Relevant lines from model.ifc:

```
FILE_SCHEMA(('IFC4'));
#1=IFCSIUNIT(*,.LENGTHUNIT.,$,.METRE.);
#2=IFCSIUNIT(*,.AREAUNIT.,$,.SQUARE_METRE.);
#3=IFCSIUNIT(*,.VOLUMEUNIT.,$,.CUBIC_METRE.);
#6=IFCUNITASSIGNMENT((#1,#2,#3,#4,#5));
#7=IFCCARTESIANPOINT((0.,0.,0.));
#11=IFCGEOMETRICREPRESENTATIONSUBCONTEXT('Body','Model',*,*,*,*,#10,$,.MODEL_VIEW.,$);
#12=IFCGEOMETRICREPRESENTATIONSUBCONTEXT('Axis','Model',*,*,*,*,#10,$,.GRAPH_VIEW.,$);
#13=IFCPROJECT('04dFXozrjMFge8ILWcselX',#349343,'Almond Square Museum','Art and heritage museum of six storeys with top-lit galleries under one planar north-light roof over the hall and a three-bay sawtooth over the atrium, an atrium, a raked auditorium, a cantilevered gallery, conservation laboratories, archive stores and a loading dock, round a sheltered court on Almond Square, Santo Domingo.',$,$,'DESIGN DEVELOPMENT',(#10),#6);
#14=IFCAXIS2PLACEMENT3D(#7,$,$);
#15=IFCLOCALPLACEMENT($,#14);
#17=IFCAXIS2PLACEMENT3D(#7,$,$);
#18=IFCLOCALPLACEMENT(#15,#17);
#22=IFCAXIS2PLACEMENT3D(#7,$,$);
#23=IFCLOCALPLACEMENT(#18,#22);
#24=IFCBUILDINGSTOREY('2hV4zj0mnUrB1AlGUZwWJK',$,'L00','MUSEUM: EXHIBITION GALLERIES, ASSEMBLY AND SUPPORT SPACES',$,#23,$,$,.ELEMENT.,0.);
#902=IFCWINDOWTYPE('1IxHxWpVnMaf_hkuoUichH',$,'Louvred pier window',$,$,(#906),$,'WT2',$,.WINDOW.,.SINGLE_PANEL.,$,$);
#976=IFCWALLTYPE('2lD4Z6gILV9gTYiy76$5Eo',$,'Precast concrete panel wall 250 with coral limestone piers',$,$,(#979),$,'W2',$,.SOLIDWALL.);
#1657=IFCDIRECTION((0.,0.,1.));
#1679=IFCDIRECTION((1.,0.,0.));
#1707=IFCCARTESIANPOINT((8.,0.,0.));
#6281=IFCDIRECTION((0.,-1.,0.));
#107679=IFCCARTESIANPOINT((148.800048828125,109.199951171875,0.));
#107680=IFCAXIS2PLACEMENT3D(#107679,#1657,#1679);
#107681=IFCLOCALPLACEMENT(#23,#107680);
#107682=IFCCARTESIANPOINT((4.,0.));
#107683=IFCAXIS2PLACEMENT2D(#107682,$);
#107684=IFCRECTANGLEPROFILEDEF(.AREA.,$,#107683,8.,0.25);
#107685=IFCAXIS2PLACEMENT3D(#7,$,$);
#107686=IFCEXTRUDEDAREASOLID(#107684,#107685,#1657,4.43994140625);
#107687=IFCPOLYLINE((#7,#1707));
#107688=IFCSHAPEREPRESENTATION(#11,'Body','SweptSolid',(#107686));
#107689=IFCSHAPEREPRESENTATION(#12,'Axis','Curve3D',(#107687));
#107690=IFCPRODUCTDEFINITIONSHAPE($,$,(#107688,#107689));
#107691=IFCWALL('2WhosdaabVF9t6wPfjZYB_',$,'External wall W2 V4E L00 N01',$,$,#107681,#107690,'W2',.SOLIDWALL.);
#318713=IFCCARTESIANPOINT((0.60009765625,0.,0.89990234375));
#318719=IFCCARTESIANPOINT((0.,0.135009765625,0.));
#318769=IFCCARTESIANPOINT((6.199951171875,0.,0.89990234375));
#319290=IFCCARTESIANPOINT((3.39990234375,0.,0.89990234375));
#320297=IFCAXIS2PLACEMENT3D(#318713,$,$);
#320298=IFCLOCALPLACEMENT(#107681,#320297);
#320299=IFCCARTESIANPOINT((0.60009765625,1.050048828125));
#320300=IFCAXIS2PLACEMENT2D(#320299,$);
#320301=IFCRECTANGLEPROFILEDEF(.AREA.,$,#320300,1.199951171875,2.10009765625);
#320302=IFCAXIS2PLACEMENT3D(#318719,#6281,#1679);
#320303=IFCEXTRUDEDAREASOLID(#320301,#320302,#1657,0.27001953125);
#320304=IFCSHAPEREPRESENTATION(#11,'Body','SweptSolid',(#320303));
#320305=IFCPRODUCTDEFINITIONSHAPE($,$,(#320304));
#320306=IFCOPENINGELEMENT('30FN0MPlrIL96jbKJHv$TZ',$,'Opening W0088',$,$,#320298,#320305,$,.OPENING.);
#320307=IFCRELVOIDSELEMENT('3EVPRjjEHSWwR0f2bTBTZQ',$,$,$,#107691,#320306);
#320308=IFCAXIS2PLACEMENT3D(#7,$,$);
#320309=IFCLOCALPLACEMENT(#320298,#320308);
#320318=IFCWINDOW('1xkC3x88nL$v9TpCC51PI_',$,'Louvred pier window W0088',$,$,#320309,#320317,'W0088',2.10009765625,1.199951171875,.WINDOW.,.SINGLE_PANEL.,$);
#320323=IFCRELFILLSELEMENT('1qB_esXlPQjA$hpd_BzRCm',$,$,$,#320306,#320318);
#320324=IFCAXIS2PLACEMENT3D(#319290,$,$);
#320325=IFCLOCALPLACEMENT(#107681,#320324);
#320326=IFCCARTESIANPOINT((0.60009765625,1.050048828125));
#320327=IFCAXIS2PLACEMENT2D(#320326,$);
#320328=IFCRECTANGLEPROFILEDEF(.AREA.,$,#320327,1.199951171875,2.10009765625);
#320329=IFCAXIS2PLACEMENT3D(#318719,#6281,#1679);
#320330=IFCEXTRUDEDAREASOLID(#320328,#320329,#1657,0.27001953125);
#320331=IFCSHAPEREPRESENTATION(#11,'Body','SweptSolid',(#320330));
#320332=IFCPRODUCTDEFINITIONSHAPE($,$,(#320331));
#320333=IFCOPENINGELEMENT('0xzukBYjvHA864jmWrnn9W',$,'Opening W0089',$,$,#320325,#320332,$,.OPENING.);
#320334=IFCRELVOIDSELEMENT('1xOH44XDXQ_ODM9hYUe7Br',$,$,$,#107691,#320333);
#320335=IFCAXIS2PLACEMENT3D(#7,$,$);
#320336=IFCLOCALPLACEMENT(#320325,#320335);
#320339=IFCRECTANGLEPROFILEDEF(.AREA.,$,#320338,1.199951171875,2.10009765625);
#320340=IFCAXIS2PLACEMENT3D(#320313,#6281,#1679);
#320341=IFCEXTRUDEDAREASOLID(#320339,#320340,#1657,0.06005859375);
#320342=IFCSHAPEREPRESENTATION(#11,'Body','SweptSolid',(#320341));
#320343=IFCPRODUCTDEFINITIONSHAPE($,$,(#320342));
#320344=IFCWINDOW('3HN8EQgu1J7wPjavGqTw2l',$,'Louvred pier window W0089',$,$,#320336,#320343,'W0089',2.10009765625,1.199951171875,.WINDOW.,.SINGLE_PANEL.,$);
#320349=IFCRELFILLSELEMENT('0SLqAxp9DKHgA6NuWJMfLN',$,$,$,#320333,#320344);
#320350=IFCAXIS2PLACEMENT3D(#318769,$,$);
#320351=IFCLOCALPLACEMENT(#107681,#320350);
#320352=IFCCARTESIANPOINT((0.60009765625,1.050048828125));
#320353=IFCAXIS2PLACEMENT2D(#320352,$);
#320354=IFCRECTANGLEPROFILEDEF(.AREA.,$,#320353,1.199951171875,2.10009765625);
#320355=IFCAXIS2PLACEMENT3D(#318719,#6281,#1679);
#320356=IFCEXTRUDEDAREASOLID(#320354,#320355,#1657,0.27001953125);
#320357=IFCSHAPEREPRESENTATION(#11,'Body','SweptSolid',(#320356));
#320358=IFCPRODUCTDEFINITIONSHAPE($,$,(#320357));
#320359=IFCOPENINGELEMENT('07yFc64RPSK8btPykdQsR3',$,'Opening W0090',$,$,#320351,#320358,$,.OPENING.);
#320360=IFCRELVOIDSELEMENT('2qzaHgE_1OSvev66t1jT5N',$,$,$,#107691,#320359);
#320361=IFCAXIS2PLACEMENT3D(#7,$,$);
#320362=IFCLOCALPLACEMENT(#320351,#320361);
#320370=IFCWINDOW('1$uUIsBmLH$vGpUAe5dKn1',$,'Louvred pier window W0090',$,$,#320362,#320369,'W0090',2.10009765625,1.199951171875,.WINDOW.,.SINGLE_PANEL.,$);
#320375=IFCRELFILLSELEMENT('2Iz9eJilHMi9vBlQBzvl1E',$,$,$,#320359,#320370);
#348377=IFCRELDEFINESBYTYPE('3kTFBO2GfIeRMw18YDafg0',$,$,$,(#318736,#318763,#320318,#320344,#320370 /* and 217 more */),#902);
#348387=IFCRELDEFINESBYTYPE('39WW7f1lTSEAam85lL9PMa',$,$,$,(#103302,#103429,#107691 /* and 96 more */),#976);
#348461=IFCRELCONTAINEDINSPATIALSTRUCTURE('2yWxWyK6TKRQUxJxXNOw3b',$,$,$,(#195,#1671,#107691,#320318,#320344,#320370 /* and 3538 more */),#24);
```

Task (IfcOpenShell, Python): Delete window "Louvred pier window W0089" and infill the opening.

```python
import ifcopenshell
import ifcopenshell.api.feature
import ifcopenshell.api.root
import ifcopenshell.geom
import ifcopenshell.util.shape

model = ifcopenshell.open("model.ifc")
settings = ifcopenshell.geom.settings()


def volume(element):
    """Net volume in cubic metres, openings subtracted."""
    shape = ifcopenshell.geom.create_shape(settings, element)
    return ifcopenshell.util.shape.get_volume(shape.geometry)


window = model.by_guid("3HN8EQgu1J7wPjavGqTw2l")
opening = window.FillsVoids[0].RelatingOpeningElement
wall = opening.VoidsElements[0].RelatingBuildingElement
before = volume(wall)

ifcopenshell.api.root.remove_product(model, product=window)
ifcopenshell.api.feature.remove_feature(model, feature=opening)

after = volume(wall)

print(f"wall volume {before:.3f} -> {after:.3f} m3")

model.write("model_rev.ifc")
```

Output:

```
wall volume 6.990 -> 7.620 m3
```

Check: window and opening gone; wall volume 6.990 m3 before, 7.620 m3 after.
